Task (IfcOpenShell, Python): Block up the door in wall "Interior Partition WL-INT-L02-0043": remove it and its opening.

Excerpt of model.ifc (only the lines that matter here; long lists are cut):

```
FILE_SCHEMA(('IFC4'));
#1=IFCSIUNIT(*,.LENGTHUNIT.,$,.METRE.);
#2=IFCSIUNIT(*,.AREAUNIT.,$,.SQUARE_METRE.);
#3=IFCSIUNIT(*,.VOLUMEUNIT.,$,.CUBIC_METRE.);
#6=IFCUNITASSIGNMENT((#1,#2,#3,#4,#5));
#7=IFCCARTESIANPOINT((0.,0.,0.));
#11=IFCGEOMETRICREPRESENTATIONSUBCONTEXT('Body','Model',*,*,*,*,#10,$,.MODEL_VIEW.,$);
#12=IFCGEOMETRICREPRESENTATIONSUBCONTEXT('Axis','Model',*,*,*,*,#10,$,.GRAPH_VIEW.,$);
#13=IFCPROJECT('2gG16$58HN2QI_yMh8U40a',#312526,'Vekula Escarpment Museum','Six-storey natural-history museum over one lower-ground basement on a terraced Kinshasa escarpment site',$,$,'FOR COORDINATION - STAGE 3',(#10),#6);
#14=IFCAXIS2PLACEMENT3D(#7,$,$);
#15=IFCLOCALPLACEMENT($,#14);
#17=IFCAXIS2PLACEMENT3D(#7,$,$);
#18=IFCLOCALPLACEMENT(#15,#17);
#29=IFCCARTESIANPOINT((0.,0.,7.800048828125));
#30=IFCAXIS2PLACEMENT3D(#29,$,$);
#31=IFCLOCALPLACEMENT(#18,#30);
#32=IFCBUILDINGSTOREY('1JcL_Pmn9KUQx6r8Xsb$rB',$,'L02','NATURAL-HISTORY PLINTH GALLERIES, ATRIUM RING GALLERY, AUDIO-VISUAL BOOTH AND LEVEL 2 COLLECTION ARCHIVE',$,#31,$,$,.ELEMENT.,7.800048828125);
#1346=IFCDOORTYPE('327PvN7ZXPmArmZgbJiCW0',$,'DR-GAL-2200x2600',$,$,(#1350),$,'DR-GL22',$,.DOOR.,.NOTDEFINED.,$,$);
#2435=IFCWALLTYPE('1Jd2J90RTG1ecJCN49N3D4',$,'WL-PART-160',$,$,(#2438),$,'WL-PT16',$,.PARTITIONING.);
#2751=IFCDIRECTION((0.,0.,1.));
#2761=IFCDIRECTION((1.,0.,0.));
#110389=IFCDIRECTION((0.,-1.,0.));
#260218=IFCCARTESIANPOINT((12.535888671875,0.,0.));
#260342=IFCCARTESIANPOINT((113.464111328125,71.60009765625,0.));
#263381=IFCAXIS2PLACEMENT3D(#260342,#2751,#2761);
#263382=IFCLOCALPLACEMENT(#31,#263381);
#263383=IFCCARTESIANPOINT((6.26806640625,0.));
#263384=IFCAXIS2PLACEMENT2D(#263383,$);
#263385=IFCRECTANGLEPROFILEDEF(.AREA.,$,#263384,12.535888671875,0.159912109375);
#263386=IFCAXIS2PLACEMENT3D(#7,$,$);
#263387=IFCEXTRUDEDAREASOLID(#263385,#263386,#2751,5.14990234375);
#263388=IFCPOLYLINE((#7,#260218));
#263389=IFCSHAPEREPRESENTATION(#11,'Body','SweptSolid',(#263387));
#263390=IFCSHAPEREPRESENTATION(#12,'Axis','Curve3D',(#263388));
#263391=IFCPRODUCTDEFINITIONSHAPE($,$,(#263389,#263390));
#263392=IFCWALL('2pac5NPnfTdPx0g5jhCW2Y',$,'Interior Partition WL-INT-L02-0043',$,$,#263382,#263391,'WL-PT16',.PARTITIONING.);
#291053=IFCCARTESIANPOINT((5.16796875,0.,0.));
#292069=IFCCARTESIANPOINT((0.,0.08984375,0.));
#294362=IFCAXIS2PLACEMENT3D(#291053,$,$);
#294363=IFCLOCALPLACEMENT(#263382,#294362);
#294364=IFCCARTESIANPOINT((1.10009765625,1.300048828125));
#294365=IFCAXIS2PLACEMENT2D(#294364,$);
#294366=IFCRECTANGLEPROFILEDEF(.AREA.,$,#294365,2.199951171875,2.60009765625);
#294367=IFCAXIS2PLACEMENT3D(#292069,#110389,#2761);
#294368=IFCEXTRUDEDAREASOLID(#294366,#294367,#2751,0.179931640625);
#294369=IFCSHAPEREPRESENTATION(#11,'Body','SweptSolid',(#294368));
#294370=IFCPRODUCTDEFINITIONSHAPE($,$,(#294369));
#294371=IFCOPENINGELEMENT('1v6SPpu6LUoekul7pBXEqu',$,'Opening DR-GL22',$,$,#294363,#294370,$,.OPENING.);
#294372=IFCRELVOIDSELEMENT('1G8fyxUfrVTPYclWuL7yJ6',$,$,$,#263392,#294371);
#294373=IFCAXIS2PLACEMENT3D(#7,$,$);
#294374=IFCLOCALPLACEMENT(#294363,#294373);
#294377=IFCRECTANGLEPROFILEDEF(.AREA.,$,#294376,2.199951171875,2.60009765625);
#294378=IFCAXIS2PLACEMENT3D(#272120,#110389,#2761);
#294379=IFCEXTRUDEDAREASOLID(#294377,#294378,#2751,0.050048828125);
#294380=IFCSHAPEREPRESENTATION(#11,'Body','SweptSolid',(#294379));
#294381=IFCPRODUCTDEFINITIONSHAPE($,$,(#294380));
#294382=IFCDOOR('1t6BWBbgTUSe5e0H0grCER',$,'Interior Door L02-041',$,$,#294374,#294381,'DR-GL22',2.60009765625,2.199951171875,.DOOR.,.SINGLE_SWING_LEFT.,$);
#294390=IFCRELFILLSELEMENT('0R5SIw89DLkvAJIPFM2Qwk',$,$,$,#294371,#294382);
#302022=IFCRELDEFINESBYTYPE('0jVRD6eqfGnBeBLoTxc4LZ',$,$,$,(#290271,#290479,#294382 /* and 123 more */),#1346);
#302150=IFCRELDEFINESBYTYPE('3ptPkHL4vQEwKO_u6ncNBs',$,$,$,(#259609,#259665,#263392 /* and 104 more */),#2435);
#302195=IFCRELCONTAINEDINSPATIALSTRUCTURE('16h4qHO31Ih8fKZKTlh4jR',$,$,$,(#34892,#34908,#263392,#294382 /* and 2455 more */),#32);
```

```python
import ifcopenshell
import ifcopenshell.api.feature
import ifcopenshell.api.root
import ifcopenshell.geom
import ifcopenshell.util.shape

model = ifcopenshell.open("model.ifc")
settings = ifcopenshell.geom.settings()


def volume(element):
    """Net volume in cubic metres, openings subtracted."""
    shape = ifcopenshell.geom.create_shape(settings, element)
    return ifcopenshell.util.shape.get_volume(shape.geometry)


door = model.by_guid("1t6BWBbgTUSe5e0H0grCER")
opening = door.FillsVoids[0].RelatingOpeningElement
wall = opening.VoidsElements[0].RelatingBuildingElement
before = volume(wall)

ifcopenshell.api.root.remove_product(model, product=door)
ifcopenshell.api.feature.remove_feature(model, feature=opening)

after = volume(wall)

print(f"wall volume {before:.3f} -> {after:.3f} m3")

model.write("model_edited.ifc")
```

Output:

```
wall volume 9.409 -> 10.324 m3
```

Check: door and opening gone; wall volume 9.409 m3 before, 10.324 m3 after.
